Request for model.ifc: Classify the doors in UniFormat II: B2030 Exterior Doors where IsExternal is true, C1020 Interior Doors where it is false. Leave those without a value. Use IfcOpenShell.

First a look at what the model holds.

```python
import ifcopenshell
import ifcopenshell.util.element

model = ifcopenshell.open("model.ifc")
print(model.schema)
print("classifications:", [c.Name for c in model.by_type("IfcClassification")])
values = [ifcopenshell.util.element.get_pset(e, "Pset_DoorCommon", "IsExternal") for e in model.by_type("IfcDoor")]
for value in (True, False, None):
    print("IsExternal", value, values.count(value))
```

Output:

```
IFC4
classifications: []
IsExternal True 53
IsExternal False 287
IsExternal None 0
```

```python
import ifcopenshell
import ifcopenshell.api.classification
import ifcopenshell.util.element

model = ifcopenshell.open("model.ifc")

system = ifcopenshell.api.classification.add_classification(model, classification="UniFormat II")

doors = model.by_type("IfcDoor")
external = {e: ifcopenshell.util.element.get_pset(e, "Pset_DoorCommon", "IsExternal") for e in doors}
for flag, code, name in ((True, "B2030", "Exterior Doors"), (False, "C1020", "Interior Doors")):
    products = [e for e in doors if external[e] is flag]
    ifcopenshell.api.classification.add_reference(
        model, products=products, classification=system, identification=code, name=name
    )
    print(code, len(products))

model.write("model_v2.ifc")
```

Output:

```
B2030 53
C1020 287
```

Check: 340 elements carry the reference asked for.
